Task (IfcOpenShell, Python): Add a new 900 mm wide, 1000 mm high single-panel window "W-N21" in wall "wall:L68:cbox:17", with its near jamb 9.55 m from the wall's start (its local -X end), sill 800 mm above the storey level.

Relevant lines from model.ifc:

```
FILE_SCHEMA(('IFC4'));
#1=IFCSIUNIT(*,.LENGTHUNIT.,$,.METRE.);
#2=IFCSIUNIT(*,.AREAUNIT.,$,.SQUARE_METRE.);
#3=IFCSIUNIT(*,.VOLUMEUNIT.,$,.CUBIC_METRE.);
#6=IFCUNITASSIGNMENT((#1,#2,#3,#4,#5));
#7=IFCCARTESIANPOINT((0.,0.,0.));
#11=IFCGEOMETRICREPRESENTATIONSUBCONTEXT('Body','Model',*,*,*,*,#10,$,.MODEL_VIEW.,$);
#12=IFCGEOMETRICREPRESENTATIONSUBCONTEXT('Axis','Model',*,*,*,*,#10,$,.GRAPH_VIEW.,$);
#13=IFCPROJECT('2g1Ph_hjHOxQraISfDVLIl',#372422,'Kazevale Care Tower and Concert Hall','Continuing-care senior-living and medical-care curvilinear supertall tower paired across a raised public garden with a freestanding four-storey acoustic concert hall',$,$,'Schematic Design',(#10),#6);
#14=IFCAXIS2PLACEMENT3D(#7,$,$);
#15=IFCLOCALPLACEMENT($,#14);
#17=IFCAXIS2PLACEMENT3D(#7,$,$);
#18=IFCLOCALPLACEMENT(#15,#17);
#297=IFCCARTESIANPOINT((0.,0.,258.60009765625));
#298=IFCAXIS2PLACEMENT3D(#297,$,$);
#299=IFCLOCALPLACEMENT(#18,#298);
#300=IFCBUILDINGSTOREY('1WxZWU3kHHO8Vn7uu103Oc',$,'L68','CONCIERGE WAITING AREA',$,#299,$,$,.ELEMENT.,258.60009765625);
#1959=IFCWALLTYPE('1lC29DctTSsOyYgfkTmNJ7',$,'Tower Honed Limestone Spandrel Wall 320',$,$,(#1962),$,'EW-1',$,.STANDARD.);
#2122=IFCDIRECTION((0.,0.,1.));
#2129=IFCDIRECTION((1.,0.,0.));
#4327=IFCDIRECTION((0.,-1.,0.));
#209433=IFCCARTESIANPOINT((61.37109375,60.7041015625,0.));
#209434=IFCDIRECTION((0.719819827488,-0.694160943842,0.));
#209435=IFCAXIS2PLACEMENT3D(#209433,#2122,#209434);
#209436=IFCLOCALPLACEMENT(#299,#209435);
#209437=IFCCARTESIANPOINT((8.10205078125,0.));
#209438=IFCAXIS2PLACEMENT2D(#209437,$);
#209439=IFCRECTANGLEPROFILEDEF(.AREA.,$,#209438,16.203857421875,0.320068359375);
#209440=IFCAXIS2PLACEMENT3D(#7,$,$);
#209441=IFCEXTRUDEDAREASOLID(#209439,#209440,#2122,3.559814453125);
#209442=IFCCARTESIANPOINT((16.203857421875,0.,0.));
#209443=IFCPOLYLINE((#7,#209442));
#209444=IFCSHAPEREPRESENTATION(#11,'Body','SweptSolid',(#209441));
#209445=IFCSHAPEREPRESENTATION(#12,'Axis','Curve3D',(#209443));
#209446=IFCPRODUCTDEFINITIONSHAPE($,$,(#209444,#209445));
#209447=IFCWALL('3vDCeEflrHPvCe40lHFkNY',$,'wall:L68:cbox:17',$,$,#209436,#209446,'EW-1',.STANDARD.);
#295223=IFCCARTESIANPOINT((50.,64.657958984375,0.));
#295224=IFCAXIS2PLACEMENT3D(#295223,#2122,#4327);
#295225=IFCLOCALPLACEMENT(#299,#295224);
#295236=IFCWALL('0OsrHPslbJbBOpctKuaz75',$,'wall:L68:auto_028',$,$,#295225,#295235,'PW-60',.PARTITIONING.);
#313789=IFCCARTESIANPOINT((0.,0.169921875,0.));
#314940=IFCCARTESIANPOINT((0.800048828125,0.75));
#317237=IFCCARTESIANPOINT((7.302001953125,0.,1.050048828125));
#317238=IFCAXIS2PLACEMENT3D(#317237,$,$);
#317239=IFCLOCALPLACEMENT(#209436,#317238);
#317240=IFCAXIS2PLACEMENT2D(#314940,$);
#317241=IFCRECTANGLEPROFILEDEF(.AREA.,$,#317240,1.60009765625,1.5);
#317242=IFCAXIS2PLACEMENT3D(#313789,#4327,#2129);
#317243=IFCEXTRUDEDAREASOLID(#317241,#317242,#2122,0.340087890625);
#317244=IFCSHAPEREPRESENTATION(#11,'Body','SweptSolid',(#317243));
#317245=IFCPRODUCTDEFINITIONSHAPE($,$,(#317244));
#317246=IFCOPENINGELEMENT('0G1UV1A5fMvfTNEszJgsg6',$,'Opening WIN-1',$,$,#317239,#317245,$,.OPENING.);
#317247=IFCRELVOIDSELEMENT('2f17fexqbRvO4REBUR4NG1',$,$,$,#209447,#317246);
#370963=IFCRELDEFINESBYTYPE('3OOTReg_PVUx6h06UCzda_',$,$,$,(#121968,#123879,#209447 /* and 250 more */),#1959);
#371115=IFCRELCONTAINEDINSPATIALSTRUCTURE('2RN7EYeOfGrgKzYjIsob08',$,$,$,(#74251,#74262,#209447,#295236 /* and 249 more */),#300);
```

```python
import numpy as np
import ifcopenshell
import ifcopenshell.api.feature
import ifcopenshell.api.geometry
import ifcopenshell.api.root
import ifcopenshell.api.spatial
import ifcopenshell.geom
import ifcopenshell.util.element
import ifcopenshell.util.placement
import ifcopenshell.util.representation
import ifcopenshell.util.shape
import ifcopenshell.util.unit

model = ifcopenshell.open("model.ifc")
unit_scale = ifcopenshell.util.unit.calculate_unit_scale(model)
settings = ifcopenshell.geom.settings()


def volume(element):
    """Net volume in cubic metres, openings subtracted."""
    shape = ifcopenshell.geom.create_shape(settings, element)
    return ifcopenshell.util.shape.get_volume(shape.geometry)


wall = model.by_guid("3vDCeEflrHPvCe40lHFkNY")
storey = ifcopenshell.util.element.get_container(wall, ifc_class="IfcBuildingStorey")
context = ifcopenshell.util.representation.get_context(model, "Model", "Body", "MODEL_VIEW")
before = volume(wall)

width, height, from_end, sill = 0.9, 1, 9.55, 0.8  # metres

# The wall runs along its own X axis, and the end named is its -X end.
wall_shape = ifcopenshell.geom.create_shape(settings, wall)
x, y, z = ifcopenshell.util.shape.get_vertices(wall_shape.geometry).T
start = x.min() + from_end
face, thickness = float(y.min()), float(y.max() - y.min())
wall_matrix = ifcopenshell.util.placement.get_local_placement(wall.ObjectPlacement)
level = ifcopenshell.util.placement.get_local_placement(storey.ObjectPlacement)[2, 3]


def in_wall(x, y):
    """Placement at x, y metres in the wall's axes, at sill height."""
    matrix = wall_matrix.copy()
    matrix[:, 3] = wall_matrix @ np.array([x / unit_scale, y / unit_scale, 0.0, 1.0])
    matrix[2, 3] = level + sill / unit_scale
    return matrix


# Opening: a box that overshoots both wall faces by 50 mm.
opening = ifcopenshell.api.root.create_entity(model, ifc_class="IfcOpeningElement", predefined_type="OPENING")
box = ifcopenshell.api.geometry.add_wall_representation(
    model, context=context, length=width, height=height, thickness=thickness + 0.1
)
ifcopenshell.api.geometry.assign_representation(model, product=opening, representation=box)
ifcopenshell.api.geometry.edit_object_placement(model, product=opening, matrix=in_wall(start, face - 0.05), is_si=False)
ifcopenshell.api.feature.add_feature(model, feature=opening, element=wall)

window = ifcopenshell.api.root.create_entity(model, ifc_class="IfcWindow", name="W-N21", predefined_type="WINDOW")
window.OverallWidth, window.OverallHeight = width / unit_scale, height / unit_scale
window.PartitioningType = "SINGLE_PANEL"
body = ifcopenshell.api.geometry.add_window_representation(
    model,
    context=context,
    overall_width=window.OverallWidth,
    overall_height=window.OverallHeight,
    partition_type="SINGLE_PANEL",
)
ifcopenshell.api.geometry.assign_representation(model, product=window, representation=body)
ifcopenshell.api.spatial.assign_container(model, products=[window], relating_structure=storey)
ifcopenshell.api.feature.add_filling(model, opening=opening, element=window)

# Centre the window in the wall's thickness.
ifcopenshell.api.geometry.edit_object_placement(model, product=window, matrix=in_wall(start, face), is_si=False)
window_shape = ifcopenshell.geom.create_shape(settings, window)
depth = ifcopenshell.util.shape.get_vertices(window_shape.geometry)[:, 1]
offset = face + thickness / 2 - (depth.min() + depth.max()) / 2
ifcopenshell.api.geometry.edit_object_placement(model, product=window, matrix=in_wall(start, offset), is_si=False)

after = volume(wall)

print(f"wall volume {before:.3f} -> {after:.3f} m3")

model.write("model_rev.ifc")
```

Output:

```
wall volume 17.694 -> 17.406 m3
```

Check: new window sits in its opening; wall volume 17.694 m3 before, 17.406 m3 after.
